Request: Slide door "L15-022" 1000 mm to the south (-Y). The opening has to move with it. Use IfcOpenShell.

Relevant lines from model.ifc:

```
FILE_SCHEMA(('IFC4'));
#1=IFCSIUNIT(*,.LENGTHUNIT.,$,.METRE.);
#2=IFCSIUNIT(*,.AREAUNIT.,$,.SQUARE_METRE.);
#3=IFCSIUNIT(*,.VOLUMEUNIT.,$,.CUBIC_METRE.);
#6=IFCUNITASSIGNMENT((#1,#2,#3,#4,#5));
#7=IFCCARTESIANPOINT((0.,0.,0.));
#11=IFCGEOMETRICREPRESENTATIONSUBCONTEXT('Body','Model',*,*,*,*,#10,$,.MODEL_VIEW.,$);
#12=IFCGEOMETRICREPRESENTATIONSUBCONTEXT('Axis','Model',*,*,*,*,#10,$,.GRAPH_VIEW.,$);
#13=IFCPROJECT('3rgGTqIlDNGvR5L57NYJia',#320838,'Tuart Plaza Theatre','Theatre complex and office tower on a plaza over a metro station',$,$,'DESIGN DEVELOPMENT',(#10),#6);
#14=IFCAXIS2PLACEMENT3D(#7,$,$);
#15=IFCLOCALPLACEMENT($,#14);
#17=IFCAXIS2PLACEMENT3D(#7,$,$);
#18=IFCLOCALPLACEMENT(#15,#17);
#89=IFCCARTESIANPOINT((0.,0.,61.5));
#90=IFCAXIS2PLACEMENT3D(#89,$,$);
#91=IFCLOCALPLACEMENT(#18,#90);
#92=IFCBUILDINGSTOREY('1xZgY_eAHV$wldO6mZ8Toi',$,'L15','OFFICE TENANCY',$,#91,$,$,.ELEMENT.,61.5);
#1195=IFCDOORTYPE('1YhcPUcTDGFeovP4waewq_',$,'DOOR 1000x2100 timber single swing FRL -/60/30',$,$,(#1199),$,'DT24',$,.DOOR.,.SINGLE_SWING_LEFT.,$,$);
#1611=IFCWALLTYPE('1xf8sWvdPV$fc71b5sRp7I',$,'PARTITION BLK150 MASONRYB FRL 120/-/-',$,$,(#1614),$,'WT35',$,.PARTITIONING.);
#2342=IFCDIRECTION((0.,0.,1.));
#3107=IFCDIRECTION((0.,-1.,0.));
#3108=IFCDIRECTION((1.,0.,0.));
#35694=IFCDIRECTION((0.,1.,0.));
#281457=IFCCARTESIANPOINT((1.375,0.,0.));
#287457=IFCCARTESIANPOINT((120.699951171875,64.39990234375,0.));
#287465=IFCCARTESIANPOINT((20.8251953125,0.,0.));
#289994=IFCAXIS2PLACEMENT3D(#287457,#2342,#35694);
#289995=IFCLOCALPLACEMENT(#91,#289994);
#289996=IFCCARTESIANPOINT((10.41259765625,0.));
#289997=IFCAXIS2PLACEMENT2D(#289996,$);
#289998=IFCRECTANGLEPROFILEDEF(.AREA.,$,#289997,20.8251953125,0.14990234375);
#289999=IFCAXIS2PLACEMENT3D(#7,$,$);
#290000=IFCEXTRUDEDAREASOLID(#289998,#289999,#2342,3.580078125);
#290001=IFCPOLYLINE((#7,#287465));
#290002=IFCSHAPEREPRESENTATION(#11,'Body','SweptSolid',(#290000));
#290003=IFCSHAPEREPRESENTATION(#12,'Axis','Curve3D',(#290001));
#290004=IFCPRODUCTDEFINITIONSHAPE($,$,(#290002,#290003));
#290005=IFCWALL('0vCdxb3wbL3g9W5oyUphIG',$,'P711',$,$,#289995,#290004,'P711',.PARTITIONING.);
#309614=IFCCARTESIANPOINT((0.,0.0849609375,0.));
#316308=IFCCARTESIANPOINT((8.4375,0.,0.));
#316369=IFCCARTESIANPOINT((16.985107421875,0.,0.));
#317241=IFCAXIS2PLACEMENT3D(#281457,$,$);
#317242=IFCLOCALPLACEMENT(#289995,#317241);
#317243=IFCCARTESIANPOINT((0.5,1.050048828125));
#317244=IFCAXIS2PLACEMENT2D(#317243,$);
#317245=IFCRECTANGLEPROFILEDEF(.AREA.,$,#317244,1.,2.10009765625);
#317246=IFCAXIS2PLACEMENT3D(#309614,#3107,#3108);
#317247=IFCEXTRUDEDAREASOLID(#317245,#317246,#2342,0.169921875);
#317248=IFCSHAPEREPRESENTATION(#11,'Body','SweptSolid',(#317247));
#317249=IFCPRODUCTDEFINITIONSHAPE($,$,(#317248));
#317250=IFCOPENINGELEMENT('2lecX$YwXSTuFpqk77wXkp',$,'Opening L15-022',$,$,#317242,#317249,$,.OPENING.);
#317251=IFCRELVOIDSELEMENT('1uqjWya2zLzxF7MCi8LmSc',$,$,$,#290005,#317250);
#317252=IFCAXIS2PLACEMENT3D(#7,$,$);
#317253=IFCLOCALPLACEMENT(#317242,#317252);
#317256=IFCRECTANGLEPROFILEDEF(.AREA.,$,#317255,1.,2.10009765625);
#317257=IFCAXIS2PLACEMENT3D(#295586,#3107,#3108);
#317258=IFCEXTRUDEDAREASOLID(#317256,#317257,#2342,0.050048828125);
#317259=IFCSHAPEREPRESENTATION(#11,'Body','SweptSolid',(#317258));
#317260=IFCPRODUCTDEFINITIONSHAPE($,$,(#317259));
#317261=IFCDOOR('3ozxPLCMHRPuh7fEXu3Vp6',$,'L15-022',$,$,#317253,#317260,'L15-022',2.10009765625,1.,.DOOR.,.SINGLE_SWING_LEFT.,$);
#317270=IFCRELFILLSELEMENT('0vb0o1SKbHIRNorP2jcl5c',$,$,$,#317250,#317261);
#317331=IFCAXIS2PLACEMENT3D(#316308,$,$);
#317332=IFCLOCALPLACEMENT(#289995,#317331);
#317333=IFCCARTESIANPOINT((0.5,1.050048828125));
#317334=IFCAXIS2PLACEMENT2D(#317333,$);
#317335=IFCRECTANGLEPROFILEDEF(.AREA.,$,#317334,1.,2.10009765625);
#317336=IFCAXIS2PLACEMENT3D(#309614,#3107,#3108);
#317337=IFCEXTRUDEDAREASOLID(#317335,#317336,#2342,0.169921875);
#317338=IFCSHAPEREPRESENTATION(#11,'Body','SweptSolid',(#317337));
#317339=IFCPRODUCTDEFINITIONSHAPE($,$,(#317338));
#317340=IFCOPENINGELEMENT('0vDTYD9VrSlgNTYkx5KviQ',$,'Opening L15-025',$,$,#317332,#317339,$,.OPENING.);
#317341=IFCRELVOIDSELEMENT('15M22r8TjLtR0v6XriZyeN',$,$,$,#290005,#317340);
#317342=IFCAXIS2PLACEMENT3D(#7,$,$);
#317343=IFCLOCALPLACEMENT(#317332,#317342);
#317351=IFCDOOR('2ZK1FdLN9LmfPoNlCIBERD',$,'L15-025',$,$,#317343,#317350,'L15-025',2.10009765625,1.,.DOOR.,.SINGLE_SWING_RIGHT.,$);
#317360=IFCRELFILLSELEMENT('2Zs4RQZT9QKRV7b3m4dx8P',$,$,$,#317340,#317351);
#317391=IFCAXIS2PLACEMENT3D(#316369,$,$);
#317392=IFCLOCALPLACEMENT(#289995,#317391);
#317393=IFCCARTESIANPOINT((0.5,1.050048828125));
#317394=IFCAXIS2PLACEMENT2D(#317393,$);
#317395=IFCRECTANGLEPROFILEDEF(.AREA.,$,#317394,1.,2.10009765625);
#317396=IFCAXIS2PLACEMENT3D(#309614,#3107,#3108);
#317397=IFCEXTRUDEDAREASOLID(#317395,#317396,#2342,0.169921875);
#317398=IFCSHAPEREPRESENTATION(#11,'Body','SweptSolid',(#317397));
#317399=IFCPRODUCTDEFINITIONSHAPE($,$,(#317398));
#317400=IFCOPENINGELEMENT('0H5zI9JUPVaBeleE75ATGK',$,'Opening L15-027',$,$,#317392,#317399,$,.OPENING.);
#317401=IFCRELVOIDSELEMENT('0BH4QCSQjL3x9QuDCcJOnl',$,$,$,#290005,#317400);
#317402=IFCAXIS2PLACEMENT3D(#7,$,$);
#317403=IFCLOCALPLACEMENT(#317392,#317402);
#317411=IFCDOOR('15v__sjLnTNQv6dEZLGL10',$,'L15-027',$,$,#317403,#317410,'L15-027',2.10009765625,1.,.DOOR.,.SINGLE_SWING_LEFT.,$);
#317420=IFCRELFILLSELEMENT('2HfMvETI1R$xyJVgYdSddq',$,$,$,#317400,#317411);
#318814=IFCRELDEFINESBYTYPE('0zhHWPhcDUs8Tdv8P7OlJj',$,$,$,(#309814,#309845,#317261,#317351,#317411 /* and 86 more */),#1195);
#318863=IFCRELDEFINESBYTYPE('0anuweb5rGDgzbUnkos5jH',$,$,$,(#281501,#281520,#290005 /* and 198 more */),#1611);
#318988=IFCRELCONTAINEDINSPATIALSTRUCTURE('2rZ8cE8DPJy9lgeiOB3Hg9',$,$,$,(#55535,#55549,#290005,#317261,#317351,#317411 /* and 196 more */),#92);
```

```python
import ifcopenshell
import ifcopenshell.api.geometry
import ifcopenshell.util.placement

model = ifcopenshell.open("model.ifc")

door = model.by_guid("3ozxPLCMHRPuh7fEXu3Vp6")
opening = door.FillsVoids[0].RelatingOpeningElement
wall = opening.VoidsElements[0].RelatingBuildingElement

wall_matrix = ifcopenshell.util.placement.get_local_placement(wall.ObjectPlacement)
shift = wall_matrix[:3, 0] * -1.0
before = ifcopenshell.util.placement.get_local_placement(door.ObjectPlacement)[:3, 3].copy()

# The door is placed relative to its opening, so it follows when the opening moves.
matrix = ifcopenshell.util.placement.get_local_placement(opening.ObjectPlacement)
matrix[:3, 3] += shift
ifcopenshell.api.geometry.edit_object_placement(
    model, product=opening, matrix=matrix, is_si=False, should_transform_children=True
)

after = ifcopenshell.util.placement.get_local_placement(door.ObjectPlacement)[:3, 3]
print("door moved by", (after - before).round(3) + 0.0)

model.write("model_rev.ifc")
```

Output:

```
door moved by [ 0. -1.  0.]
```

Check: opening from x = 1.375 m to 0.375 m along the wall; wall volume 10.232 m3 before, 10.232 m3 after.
